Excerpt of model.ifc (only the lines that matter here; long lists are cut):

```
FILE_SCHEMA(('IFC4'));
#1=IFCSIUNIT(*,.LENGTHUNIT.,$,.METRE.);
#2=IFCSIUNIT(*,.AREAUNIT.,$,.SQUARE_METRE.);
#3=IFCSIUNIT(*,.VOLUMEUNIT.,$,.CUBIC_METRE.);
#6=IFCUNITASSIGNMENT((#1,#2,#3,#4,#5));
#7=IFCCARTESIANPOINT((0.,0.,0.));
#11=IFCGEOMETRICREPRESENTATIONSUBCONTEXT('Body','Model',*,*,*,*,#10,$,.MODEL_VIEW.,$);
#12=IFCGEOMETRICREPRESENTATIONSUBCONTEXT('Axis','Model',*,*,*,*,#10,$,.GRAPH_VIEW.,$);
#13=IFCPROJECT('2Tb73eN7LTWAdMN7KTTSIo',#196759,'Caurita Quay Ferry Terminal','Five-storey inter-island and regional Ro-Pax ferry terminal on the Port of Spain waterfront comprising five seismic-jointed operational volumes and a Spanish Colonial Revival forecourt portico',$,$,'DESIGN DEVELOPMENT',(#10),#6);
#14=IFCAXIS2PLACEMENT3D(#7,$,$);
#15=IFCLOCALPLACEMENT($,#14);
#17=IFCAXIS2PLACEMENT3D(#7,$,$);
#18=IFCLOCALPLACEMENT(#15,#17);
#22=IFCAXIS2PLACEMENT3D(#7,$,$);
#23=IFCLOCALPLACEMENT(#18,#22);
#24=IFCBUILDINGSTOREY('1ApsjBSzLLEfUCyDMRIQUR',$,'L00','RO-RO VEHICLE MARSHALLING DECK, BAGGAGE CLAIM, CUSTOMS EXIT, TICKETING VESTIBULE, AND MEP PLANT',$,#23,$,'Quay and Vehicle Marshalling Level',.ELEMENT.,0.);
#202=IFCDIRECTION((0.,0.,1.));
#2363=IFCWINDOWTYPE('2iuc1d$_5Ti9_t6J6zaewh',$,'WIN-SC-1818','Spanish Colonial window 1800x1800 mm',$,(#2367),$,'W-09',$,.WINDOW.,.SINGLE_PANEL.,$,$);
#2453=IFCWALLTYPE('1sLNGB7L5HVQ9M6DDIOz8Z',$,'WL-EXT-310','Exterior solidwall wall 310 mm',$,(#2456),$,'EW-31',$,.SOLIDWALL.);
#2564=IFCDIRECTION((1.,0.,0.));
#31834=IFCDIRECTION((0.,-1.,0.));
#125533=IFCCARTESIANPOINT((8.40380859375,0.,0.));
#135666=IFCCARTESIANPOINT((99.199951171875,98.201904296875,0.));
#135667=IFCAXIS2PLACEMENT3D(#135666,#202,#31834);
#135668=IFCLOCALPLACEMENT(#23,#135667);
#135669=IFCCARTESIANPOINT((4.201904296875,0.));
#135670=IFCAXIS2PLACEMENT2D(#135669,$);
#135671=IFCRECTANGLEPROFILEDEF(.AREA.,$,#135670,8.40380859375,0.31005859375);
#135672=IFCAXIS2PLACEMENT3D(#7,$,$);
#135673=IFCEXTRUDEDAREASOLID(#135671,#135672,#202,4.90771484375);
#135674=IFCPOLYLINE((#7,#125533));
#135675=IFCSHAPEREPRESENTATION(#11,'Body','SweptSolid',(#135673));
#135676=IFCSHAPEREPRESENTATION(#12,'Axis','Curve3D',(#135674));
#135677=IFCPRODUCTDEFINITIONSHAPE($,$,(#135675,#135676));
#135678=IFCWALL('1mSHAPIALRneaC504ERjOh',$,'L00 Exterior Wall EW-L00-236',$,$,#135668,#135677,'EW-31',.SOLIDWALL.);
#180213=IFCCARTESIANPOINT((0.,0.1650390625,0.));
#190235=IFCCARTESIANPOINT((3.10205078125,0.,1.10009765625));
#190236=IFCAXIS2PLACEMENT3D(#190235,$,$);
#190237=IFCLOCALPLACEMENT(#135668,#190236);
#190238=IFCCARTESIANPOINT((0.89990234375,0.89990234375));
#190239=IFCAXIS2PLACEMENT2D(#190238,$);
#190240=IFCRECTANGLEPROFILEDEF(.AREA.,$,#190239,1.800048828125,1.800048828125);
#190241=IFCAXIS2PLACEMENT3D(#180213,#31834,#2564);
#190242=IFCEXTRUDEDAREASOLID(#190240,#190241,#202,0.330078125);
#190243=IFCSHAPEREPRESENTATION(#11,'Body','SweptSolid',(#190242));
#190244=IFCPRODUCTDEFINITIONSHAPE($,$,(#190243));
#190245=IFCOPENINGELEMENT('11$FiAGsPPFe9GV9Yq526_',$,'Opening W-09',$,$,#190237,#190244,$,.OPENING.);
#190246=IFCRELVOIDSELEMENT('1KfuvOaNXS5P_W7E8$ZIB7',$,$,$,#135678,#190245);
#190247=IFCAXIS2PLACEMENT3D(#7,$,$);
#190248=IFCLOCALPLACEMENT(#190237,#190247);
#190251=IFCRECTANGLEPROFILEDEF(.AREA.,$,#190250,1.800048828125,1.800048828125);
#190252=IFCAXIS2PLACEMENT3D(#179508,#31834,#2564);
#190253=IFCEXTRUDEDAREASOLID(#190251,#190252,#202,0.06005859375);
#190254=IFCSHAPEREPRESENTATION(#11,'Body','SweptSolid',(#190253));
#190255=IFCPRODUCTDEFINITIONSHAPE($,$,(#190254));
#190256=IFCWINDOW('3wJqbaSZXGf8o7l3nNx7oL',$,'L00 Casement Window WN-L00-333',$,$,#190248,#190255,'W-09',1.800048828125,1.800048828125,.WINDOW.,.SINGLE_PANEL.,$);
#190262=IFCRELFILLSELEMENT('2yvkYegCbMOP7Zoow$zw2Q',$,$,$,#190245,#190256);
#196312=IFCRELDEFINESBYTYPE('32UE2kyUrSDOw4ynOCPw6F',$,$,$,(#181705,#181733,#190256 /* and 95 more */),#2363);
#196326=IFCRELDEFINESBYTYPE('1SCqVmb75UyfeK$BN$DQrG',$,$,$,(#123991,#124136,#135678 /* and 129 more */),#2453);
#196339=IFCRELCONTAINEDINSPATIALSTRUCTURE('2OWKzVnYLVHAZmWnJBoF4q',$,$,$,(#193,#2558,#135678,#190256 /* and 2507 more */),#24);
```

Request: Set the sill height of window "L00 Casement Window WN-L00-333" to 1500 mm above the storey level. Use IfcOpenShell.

```python
import numpy as np
import ifcopenshell
import ifcopenshell.api.geometry
import ifcopenshell.geom
import ifcopenshell.util.element
import ifcopenshell.util.placement
import ifcopenshell.util.shape
import ifcopenshell.util.unit

model = ifcopenshell.open("model.ifc")
unit_scale = ifcopenshell.util.unit.calculate_unit_scale(model)

window = model.by_guid("3wJqbaSZXGf8o7l3nNx7oL")
opening = window.FillsVoids[0].RelatingOpeningElement
storey = ifcopenshell.util.element.get_container(window, ifc_class="IfcBuildingStorey")
level = ifcopenshell.util.placement.get_local_placement(storey.ObjectPlacement)[2, 3]

# The opening's origin need not be at the sill, so measure its lowest point.
shape = ifcopenshell.geom.create_shape(ifcopenshell.geom.settings(), opening)
bottom = ifcopenshell.util.shape.get_shape_bottom_elevation(shape, shape.geometry) / unit_scale
dz = level + 1.5 / unit_scale - bottom

shift = np.array([0.0, 0.0, dz])
# The window is placed relative to its opening, so it follows when the opening moves.
matrix = ifcopenshell.util.placement.get_local_placement(opening.ObjectPlacement)
matrix[:3, 3] += shift
ifcopenshell.api.geometry.edit_object_placement(
    model, product=opening, matrix=matrix, is_si=False, should_transform_children=True
)

print(f"moved by {dz * unit_scale:+.3f} m")

model.write("model_v2.ifc")
```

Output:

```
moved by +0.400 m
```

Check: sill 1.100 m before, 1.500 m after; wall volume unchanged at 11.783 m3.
